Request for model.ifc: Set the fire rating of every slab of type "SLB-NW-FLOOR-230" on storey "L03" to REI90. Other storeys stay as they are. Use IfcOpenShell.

First a look at what the model holds.

```python
import ifcopenshell
import ifcopenshell.util.element

model = ifcopenshell.open("model.ifc")
print(model.schema)
storey = next(s for s in model.by_type("IfcBuildingStorey") if s.Name == "L03")
slabs = [e for e in ifcopenshell.util.element.get_decomposition(storey) if e.is_a("IfcSlab")]
seen = {}
for e in slabs:
    element_type = ifcopenshell.util.element.get_type(e)
    key = (element_type.Name if element_type != e and element_type else None, ifcopenshell.util.element.get_pset(e, "Pset_SlabCommon", "FireRating"))
    seen[key] = seen.get(key, 0) + 1
for (name, value), count in sorted(seen.items(), key=str):
    print(count, "x", name, "|", value)
```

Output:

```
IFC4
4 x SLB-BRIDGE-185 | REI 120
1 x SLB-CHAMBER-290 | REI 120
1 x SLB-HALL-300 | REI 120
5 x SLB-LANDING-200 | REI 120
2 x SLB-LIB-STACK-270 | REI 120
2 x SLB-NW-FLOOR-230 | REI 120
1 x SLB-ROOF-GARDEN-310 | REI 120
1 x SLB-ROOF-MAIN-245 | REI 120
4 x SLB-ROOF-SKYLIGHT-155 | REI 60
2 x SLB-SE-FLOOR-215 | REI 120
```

```python
import ifcopenshell
import ifcopenshell.api.pset
import ifcopenshell.util.element

model = ifcopenshell.open("model.ifc")

storey = next(s for s in model.by_type("IfcBuildingStorey") if s.Name == "L03")
slabs = [e for e in ifcopenshell.util.element.get_decomposition(storey) if e.is_a("IfcSlab")]

count = 0
for e in slabs:
    element_type = ifcopenshell.util.element.get_type(e)
    if element_type in (None, e) or element_type.Name != "SLB-NW-FLOOR-230":
        continue
    # add_pset returns the element's existing set when there is one.
    pset = ifcopenshell.api.pset.add_pset(model, product=e, name="Pset_SlabCommon")
    ifcopenshell.api.pset.edit_pset(model, pset=pset, properties={"FireRating": "REI90"})
    count += 1

print(count, "slabs updated")

model.write("model-out.ifc")
```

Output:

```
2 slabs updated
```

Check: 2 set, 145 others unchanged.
